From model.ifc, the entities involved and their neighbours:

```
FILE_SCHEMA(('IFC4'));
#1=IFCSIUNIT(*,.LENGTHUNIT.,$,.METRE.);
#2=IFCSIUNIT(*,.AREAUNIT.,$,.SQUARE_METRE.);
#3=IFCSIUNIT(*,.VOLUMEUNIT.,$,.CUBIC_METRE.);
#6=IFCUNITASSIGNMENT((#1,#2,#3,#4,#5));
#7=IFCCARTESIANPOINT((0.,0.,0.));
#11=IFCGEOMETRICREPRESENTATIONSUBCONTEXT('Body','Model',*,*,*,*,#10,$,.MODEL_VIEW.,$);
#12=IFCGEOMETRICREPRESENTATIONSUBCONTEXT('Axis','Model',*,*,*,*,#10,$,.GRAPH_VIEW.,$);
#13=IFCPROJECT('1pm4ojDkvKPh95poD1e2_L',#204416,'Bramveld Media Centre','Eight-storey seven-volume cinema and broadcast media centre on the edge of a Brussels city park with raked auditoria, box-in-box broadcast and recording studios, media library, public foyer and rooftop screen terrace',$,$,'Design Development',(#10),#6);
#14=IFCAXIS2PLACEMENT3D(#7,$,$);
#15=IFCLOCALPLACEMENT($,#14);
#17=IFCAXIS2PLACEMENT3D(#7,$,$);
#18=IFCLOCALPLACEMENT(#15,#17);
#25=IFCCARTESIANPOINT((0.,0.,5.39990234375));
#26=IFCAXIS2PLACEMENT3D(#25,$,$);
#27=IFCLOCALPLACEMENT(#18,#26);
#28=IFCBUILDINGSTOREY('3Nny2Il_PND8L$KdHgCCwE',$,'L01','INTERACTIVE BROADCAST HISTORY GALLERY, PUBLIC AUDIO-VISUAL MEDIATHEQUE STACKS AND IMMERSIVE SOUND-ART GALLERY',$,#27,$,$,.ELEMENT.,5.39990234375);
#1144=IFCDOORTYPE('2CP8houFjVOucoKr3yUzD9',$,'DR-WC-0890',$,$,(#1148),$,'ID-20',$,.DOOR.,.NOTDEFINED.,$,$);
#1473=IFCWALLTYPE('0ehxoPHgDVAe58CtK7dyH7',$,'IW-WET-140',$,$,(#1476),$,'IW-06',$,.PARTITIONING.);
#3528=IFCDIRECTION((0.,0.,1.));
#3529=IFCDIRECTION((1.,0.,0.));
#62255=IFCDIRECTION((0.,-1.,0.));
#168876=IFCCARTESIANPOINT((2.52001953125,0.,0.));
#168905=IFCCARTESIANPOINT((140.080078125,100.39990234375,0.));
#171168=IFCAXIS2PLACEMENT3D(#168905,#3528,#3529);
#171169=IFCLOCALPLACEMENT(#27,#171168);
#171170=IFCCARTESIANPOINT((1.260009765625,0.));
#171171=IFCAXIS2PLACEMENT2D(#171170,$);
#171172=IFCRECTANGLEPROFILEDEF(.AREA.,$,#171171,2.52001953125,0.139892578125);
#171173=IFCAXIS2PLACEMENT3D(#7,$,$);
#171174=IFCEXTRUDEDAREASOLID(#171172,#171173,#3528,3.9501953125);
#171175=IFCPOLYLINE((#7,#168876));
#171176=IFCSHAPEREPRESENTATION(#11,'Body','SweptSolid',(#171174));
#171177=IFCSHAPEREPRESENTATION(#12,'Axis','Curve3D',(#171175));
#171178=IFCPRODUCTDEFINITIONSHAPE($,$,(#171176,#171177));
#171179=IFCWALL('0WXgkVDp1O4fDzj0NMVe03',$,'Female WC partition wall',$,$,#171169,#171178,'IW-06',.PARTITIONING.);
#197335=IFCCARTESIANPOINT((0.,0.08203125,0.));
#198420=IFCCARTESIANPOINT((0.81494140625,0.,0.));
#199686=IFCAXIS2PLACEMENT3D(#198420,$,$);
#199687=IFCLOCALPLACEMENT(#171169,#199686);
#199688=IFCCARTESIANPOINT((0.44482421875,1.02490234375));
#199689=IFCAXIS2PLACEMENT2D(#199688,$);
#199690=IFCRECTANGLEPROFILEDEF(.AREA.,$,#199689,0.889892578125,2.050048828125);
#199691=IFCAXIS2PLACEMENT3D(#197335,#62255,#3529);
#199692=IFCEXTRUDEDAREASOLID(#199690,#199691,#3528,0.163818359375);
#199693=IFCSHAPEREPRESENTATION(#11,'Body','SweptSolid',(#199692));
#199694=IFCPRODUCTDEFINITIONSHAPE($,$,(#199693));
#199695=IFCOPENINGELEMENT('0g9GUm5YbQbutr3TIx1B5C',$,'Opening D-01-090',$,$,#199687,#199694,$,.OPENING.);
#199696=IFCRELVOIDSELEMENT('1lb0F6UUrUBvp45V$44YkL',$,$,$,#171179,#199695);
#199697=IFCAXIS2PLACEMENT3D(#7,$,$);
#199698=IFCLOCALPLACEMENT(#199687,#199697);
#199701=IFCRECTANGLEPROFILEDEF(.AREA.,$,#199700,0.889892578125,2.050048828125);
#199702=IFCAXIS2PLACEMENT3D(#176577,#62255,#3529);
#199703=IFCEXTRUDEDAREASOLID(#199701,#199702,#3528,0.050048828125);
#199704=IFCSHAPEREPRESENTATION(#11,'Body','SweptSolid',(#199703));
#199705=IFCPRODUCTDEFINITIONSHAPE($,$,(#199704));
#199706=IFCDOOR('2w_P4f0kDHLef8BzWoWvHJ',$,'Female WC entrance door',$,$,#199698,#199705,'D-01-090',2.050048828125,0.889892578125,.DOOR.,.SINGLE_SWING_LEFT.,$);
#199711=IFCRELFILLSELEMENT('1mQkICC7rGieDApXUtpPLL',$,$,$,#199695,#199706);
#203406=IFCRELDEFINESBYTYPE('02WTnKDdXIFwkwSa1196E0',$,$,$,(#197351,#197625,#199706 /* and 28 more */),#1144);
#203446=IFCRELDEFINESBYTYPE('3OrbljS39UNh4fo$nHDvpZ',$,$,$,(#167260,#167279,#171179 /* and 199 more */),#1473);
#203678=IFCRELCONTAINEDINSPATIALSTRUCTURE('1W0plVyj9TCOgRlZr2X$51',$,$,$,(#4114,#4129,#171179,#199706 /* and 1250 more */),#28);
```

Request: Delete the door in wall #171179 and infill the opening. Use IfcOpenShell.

```python
import ifcopenshell
import ifcopenshell.api.feature
import ifcopenshell.api.root
import ifcopenshell.geom
import ifcopenshell.util.shape

model = ifcopenshell.open("model.ifc")
settings = ifcopenshell.geom.settings()


def volume(element):
    """Net volume in cubic metres, openings subtracted."""
    shape = ifcopenshell.geom.create_shape(settings, element)
    return ifcopenshell.util.shape.get_volume(shape.geometry)


door = model.by_guid("2w_P4f0kDHLef8BzWoWvHJ")
opening = door.FillsVoids[0].RelatingOpeningElement
wall = opening.VoidsElements[0].RelatingBuildingElement
before = volume(wall)

ifcopenshell.api.root.remove_product(model, product=door)
ifcopenshell.api.feature.remove_feature(model, feature=opening)

after = volume(wall)

print(f"wall volume {before:.3f} -> {after:.3f} m3")

model.write("model_updated.ifc")
```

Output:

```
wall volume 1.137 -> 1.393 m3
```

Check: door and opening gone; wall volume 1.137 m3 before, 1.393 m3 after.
